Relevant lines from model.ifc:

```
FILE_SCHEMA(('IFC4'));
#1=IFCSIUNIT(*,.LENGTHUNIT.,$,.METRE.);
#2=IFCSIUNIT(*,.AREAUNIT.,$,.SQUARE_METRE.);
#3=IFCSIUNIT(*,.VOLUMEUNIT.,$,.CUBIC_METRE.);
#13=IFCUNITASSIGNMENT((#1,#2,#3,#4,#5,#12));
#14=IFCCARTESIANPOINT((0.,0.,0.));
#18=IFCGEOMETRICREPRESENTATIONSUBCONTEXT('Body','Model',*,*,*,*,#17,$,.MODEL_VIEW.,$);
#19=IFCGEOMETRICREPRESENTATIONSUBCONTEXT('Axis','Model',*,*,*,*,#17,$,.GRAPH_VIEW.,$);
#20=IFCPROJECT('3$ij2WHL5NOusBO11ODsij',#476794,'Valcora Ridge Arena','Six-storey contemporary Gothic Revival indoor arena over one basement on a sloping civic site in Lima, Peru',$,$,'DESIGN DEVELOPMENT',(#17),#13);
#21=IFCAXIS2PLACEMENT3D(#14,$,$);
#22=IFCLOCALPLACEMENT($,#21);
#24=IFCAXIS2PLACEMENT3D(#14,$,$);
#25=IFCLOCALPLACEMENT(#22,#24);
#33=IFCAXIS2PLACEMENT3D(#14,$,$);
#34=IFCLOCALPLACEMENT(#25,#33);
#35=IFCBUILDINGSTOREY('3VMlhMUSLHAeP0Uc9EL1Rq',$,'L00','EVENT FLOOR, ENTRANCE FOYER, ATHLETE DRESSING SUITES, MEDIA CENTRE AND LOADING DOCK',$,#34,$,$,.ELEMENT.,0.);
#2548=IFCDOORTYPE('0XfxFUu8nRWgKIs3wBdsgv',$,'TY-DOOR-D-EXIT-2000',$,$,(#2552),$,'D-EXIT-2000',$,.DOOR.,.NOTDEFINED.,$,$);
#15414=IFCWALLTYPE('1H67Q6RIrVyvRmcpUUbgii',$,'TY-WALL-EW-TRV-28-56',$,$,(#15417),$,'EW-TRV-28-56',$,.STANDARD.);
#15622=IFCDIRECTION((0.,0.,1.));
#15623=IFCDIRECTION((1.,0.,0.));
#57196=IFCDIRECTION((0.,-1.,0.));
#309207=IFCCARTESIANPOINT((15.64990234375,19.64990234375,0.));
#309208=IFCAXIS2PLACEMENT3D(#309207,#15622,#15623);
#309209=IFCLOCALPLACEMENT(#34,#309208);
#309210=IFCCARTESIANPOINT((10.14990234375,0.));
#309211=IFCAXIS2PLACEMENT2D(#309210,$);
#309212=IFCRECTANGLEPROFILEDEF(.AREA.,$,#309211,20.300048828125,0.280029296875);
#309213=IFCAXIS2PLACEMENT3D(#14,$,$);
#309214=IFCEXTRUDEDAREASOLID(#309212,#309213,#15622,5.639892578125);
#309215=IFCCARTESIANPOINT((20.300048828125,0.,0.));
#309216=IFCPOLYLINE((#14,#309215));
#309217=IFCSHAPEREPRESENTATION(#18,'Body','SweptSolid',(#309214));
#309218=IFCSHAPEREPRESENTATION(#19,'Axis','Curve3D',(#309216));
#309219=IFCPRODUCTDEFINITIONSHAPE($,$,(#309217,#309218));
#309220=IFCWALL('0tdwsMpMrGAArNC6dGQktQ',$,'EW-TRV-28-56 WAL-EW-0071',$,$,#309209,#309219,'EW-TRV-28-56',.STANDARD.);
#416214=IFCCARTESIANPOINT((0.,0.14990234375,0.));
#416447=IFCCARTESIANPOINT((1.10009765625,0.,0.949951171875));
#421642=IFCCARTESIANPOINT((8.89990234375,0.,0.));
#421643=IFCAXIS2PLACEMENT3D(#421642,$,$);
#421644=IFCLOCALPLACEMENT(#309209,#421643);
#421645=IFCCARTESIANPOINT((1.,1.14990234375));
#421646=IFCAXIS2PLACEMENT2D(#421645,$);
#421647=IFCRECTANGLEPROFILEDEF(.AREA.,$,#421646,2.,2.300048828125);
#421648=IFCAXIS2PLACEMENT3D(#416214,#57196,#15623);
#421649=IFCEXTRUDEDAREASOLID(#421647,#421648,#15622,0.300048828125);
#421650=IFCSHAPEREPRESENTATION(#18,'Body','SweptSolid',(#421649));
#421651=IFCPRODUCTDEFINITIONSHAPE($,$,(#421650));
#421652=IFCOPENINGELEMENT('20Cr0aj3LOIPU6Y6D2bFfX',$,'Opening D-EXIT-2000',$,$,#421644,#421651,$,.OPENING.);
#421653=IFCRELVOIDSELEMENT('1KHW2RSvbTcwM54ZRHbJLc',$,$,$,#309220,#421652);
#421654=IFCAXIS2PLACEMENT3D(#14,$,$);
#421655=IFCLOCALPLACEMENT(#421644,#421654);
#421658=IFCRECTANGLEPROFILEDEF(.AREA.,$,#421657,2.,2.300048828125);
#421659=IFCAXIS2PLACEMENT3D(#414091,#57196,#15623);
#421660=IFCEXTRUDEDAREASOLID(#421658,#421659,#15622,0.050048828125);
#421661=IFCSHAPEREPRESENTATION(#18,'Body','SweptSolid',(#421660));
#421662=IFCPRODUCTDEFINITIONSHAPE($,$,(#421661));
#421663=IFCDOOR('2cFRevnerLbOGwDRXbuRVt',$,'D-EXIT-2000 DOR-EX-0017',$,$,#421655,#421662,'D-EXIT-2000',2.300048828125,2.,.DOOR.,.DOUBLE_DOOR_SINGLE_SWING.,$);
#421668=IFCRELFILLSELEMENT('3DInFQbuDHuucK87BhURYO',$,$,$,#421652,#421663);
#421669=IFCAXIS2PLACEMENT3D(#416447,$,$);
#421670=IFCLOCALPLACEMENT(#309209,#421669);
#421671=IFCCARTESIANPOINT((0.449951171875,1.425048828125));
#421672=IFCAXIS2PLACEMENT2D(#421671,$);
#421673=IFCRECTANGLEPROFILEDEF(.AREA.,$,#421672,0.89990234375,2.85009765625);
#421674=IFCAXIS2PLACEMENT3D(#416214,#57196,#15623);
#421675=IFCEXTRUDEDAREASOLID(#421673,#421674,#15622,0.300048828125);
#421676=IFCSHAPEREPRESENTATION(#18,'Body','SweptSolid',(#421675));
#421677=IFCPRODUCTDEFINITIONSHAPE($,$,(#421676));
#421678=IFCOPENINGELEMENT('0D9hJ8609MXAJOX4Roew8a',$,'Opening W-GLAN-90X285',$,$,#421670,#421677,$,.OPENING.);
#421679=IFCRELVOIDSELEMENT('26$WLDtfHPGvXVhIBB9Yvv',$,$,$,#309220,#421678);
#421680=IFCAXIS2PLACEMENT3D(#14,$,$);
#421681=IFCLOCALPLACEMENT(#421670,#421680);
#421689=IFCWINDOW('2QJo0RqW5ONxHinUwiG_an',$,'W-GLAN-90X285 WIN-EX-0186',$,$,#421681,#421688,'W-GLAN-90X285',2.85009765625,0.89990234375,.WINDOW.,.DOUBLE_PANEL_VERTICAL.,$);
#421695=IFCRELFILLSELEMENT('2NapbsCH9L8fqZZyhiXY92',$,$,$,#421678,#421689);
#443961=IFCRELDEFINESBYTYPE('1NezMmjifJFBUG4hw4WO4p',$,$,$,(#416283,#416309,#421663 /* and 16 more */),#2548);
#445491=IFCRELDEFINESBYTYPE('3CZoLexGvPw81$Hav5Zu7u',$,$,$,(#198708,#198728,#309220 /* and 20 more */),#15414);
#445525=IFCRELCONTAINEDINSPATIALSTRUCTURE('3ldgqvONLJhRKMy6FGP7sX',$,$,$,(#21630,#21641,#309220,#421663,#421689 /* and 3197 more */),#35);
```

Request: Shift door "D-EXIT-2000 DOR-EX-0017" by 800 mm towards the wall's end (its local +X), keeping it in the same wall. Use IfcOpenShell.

```python
import ifcopenshell
import ifcopenshell.api.geometry
import ifcopenshell.util.placement

model = ifcopenshell.open("model.ifc")

door = model.by_guid("2cFRevnerLbOGwDRXbuRVt")
opening = door.FillsVoids[0].RelatingOpeningElement
wall = opening.VoidsElements[0].RelatingBuildingElement

wall_matrix = ifcopenshell.util.placement.get_local_placement(wall.ObjectPlacement)
shift = wall_matrix[:3, 0] * 0.8
before = ifcopenshell.util.placement.get_local_placement(door.ObjectPlacement)[:3, 3].copy()

# The door is placed relative to its opening, so it follows when the opening moves.
matrix = ifcopenshell.util.placement.get_local_placement(opening.ObjectPlacement)
matrix[:3, 3] += shift
ifcopenshell.api.geometry.edit_object_placement(
    model, product=opening, matrix=matrix, is_si=False, should_transform_children=True
)

after = ifcopenshell.util.placement.get_local_placement(door.ObjectPlacement)[:3, 3]
print("door moved by", (after - before).round(3) + 0.0)

model.write("model_v2.ifc")
```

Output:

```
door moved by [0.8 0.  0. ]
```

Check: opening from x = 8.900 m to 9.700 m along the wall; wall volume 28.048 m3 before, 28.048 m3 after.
